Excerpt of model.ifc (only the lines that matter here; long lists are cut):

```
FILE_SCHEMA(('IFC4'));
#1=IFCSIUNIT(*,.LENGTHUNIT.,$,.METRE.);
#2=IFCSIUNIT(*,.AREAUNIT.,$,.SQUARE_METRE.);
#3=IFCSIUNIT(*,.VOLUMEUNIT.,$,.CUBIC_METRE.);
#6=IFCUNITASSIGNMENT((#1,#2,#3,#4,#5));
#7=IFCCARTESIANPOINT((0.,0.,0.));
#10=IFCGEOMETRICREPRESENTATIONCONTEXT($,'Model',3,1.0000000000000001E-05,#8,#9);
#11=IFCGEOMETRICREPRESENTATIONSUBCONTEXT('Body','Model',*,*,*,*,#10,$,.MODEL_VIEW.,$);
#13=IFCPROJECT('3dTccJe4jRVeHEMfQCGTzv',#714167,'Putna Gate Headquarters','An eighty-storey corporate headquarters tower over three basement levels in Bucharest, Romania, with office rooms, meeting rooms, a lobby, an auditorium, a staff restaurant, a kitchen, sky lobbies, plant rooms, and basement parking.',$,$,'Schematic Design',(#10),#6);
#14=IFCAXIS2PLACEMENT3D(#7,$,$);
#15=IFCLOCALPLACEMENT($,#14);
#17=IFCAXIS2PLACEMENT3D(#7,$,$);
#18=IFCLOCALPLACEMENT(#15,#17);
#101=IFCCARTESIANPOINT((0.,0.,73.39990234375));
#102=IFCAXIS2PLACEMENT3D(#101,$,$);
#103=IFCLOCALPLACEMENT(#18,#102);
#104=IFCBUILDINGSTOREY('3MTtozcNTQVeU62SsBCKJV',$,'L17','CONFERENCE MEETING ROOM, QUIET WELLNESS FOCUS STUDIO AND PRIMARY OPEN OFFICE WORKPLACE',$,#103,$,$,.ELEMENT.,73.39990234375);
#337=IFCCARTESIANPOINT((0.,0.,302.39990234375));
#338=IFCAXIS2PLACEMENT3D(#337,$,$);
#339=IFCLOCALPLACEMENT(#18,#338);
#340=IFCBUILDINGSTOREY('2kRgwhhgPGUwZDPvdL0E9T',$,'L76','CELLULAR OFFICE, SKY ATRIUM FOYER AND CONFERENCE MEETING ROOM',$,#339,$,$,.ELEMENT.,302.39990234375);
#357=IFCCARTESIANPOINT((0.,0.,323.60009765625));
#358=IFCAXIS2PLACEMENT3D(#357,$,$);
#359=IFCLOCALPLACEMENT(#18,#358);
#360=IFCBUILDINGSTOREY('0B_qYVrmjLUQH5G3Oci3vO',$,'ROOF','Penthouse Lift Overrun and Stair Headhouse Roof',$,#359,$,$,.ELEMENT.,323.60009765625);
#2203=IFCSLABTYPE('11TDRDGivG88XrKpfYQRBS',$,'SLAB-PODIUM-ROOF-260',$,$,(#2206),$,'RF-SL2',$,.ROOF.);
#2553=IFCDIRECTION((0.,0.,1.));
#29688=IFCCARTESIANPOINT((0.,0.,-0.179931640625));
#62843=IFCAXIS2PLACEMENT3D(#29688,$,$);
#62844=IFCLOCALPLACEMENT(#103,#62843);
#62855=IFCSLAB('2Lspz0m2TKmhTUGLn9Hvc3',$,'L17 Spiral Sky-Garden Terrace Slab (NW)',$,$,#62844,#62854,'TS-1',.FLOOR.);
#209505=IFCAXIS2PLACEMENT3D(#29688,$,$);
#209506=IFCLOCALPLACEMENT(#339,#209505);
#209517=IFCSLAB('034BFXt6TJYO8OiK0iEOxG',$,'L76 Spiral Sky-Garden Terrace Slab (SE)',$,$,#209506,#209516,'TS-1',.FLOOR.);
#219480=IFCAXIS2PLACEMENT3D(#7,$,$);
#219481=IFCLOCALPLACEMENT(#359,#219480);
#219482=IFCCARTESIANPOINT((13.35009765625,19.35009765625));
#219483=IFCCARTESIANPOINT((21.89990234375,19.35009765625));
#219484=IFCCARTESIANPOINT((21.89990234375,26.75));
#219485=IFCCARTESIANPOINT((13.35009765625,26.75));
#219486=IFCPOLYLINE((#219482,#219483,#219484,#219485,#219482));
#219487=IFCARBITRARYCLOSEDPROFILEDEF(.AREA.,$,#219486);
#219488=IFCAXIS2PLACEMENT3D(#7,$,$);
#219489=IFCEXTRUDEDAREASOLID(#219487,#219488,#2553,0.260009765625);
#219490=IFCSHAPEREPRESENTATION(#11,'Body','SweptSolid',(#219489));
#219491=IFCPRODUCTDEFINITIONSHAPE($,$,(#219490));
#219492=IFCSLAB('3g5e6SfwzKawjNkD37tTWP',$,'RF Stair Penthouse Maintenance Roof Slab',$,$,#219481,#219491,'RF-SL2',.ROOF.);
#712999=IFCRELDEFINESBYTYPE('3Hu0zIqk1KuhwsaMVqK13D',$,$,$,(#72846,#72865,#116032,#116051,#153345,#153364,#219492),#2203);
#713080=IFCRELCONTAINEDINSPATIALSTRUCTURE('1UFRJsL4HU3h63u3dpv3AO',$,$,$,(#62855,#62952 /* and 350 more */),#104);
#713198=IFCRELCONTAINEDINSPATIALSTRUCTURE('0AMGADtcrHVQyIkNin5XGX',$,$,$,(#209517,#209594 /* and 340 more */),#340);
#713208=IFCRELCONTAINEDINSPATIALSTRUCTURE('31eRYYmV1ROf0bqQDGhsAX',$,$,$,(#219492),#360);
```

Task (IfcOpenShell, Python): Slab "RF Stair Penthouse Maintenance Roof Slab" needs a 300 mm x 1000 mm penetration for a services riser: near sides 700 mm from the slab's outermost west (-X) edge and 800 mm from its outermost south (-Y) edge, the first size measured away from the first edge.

```python
import numpy as np
import ifcopenshell
import ifcopenshell.api.feature
import ifcopenshell.api.geometry
import ifcopenshell.api.root
import ifcopenshell.geom
import ifcopenshell.util.placement
import ifcopenshell.util.representation
import ifcopenshell.util.shape
import ifcopenshell.util.unit

model = ifcopenshell.open("model.ifc")
unit_scale = ifcopenshell.util.unit.calculate_unit_scale(model)
settings = ifcopenshell.geom.settings()


def volume(element):
    """Net volume in cubic metres, openings subtracted."""
    shape = ifcopenshell.geom.create_shape(settings, element)
    return ifcopenshell.util.shape.get_volume(shape.geometry)


slab = model.by_guid("3g5e6SfwzKawjNkD37tTWP")
before = volume(slab)

# Extent in the slab's own axes, in metres. The edges named are its -X and -Y sides.
slab_shape = ifcopenshell.geom.create_shape(settings, slab)
vertices = ifcopenshell.util.shape.get_vertices(slab_shape.geometry)
x_min, y_min, bottom = vertices.min(axis=0)
top = vertices[:, 2].max()

opening = ifcopenshell.api.root.create_entity(model, ifc_class="IfcOpeningElement", name="Services riser opening", predefined_type="OPENING")
context = ifcopenshell.util.representation.get_context(model, "Model", "Body", "MODEL_VIEW")
width, depth = 0.3, 1
outline = [(0.0, 0.0), (width, 0.0), (width, depth), (0.0, depth), (0.0, 0.0)]
# Overshoot both faces by 50 mm so the cut is clean.
shape = ifcopenshell.api.geometry.add_slab_representation(
    model, context=context, depth=top - bottom + 0.1, polyline=outline
)
ifcopenshell.api.geometry.assign_representation(model, product=opening, representation=shape)

matrix = ifcopenshell.util.placement.get_local_placement(slab.ObjectPlacement)
matrix[:, 3] = matrix @ np.append(np.array([x_min + 0.7, y_min + 0.8, bottom - 0.05]) / unit_scale, 1.0)
ifcopenshell.api.geometry.edit_object_placement(model, product=opening, matrix=matrix, is_si=False)
ifcopenshell.api.feature.add_feature(model, feature=opening, element=slab)

after = volume(slab)

print(f"slab volume {before:.3f} -> {after:.3f} m3")

model.write("model-out.ifc")
```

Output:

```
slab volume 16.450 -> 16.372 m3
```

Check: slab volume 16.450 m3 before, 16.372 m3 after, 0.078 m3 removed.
